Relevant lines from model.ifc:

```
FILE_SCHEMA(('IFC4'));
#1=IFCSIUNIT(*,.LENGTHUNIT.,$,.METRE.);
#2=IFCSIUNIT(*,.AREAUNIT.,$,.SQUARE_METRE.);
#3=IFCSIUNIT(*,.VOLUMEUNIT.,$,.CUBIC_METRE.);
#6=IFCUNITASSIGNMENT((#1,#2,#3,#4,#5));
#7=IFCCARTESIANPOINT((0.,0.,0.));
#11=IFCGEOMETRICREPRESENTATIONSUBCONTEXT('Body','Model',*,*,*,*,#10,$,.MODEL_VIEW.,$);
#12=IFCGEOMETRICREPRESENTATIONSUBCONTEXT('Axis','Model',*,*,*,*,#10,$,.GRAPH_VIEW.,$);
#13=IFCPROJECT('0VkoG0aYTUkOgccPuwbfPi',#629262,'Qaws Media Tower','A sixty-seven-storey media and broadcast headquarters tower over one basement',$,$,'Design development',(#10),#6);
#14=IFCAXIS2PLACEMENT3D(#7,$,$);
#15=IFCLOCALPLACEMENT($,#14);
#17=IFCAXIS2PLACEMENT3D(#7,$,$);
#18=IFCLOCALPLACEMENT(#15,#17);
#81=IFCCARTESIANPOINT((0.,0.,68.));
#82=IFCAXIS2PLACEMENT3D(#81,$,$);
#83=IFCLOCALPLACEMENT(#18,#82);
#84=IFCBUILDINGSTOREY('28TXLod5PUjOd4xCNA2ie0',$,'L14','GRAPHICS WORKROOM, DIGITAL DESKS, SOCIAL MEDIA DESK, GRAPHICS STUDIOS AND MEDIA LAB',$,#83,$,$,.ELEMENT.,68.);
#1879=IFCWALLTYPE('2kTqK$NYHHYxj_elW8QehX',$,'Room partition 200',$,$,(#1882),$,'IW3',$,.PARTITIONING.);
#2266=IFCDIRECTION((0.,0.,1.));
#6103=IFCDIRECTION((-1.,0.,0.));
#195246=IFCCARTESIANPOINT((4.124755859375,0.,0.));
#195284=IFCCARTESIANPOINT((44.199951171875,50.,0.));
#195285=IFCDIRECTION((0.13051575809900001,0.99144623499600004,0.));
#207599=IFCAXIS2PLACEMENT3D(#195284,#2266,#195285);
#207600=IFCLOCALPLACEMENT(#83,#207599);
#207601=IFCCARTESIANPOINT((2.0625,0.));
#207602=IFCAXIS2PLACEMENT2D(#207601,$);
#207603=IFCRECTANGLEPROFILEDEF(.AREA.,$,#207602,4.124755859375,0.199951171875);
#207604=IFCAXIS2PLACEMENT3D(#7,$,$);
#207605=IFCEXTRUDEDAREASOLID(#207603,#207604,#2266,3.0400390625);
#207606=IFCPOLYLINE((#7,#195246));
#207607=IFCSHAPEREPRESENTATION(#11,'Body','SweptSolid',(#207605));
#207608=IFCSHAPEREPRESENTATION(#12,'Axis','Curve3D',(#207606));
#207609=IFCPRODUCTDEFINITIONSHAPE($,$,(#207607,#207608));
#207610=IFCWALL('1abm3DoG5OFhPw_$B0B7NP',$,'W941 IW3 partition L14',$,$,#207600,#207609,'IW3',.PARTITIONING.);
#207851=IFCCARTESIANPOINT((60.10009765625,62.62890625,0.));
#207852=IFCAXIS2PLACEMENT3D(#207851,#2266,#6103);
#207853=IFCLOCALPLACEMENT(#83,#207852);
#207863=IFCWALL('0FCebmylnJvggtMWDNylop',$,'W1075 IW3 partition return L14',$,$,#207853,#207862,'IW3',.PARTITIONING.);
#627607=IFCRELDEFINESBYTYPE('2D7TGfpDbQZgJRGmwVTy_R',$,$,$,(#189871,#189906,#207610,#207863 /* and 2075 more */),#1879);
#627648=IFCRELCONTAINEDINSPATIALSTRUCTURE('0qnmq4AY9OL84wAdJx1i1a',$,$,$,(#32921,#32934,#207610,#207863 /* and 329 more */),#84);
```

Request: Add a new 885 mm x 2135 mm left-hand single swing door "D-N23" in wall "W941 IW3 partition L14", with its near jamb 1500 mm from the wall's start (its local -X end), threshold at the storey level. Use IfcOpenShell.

```python
import numpy as np
import ifcopenshell
import ifcopenshell.api.feature
import ifcopenshell.api.geometry
import ifcopenshell.api.root
import ifcopenshell.api.spatial
import ifcopenshell.geom
import ifcopenshell.util.element
import ifcopenshell.util.placement
import ifcopenshell.util.representation
import ifcopenshell.util.shape
import ifcopenshell.util.unit

model = ifcopenshell.open("model.ifc")
unit_scale = ifcopenshell.util.unit.calculate_unit_scale(model)
settings = ifcopenshell.geom.settings()


def volume(element):
    """Net volume in cubic metres, openings subtracted."""
    shape = ifcopenshell.geom.create_shape(settings, element)
    return ifcopenshell.util.shape.get_volume(shape.geometry)


wall = model.by_guid("1abm3DoG5OFhPw_$B0B7NP")
storey = ifcopenshell.util.element.get_container(wall, ifc_class="IfcBuildingStorey")
context = ifcopenshell.util.representation.get_context(model, "Model", "Body", "MODEL_VIEW")
before = volume(wall)

width, height, from_end, sill = 0.885, 2.135, 1.5, 0.0  # metres

# The wall runs along its own X axis, and the end named is its -X end.
wall_shape = ifcopenshell.geom.create_shape(settings, wall)
x, y, z = ifcopenshell.util.shape.get_vertices(wall_shape.geometry).T
start = x.min() + from_end
face, thickness = float(y.min()), float(y.max() - y.min())
wall_matrix = ifcopenshell.util.placement.get_local_placement(wall.ObjectPlacement)
level = ifcopenshell.util.placement.get_local_placement(storey.ObjectPlacement)[2, 3]


def in_wall(x, y):
    """Placement at x, y metres in the wall's axes, at sill height."""
    matrix = wall_matrix.copy()
    matrix[:, 3] = wall_matrix @ np.array([x / unit_scale, y / unit_scale, 0.0, 1.0])
    matrix[2, 3] = level + sill / unit_scale
    return matrix


# Opening: a box that overshoots both wall faces by 50 mm.
opening = ifcopenshell.api.root.create_entity(model, ifc_class="IfcOpeningElement", predefined_type="OPENING")
box = ifcopenshell.api.geometry.add_wall_representation(
    model, context=context, length=width, height=height, thickness=thickness + 0.1
)
ifcopenshell.api.geometry.assign_representation(model, product=opening, representation=box)
ifcopenshell.api.geometry.edit_object_placement(model, product=opening, matrix=in_wall(start, face - 0.05), is_si=False)
ifcopenshell.api.feature.add_feature(model, feature=opening, element=wall)

door = ifcopenshell.api.root.create_entity(model, ifc_class="IfcDoor", name="D-N23", predefined_type="DOOR")
door.OverallWidth, door.OverallHeight = width / unit_scale, height / unit_scale
door.OperationType = "SINGLE_SWING_LEFT"
body = ifcopenshell.api.geometry.add_door_representation(
    model,
    context=context,
    overall_width=door.OverallWidth,
    overall_height=door.OverallHeight,
    operation_type="SINGLE_SWING_LEFT",
    lining_properties={"LiningDepth": thickness / unit_scale, "ThresholdDepth": thickness / unit_scale},
)
ifcopenshell.api.geometry.assign_representation(model, product=door, representation=body)
ifcopenshell.api.spatial.assign_container(model, products=[door], relating_structure=storey)
ifcopenshell.api.feature.add_filling(model, opening=opening, element=door)

# The lining spans the wall, so the door starts at the wall face.
ifcopenshell.api.geometry.edit_object_placement(model, product=door, matrix=in_wall(start, face), is_si=False)

after = volume(wall)

print(f"wall volume {before:.3f} -> {after:.3f} m3")

model.write("model_edited.ifc")
```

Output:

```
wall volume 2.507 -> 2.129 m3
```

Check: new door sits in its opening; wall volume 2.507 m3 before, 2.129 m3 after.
